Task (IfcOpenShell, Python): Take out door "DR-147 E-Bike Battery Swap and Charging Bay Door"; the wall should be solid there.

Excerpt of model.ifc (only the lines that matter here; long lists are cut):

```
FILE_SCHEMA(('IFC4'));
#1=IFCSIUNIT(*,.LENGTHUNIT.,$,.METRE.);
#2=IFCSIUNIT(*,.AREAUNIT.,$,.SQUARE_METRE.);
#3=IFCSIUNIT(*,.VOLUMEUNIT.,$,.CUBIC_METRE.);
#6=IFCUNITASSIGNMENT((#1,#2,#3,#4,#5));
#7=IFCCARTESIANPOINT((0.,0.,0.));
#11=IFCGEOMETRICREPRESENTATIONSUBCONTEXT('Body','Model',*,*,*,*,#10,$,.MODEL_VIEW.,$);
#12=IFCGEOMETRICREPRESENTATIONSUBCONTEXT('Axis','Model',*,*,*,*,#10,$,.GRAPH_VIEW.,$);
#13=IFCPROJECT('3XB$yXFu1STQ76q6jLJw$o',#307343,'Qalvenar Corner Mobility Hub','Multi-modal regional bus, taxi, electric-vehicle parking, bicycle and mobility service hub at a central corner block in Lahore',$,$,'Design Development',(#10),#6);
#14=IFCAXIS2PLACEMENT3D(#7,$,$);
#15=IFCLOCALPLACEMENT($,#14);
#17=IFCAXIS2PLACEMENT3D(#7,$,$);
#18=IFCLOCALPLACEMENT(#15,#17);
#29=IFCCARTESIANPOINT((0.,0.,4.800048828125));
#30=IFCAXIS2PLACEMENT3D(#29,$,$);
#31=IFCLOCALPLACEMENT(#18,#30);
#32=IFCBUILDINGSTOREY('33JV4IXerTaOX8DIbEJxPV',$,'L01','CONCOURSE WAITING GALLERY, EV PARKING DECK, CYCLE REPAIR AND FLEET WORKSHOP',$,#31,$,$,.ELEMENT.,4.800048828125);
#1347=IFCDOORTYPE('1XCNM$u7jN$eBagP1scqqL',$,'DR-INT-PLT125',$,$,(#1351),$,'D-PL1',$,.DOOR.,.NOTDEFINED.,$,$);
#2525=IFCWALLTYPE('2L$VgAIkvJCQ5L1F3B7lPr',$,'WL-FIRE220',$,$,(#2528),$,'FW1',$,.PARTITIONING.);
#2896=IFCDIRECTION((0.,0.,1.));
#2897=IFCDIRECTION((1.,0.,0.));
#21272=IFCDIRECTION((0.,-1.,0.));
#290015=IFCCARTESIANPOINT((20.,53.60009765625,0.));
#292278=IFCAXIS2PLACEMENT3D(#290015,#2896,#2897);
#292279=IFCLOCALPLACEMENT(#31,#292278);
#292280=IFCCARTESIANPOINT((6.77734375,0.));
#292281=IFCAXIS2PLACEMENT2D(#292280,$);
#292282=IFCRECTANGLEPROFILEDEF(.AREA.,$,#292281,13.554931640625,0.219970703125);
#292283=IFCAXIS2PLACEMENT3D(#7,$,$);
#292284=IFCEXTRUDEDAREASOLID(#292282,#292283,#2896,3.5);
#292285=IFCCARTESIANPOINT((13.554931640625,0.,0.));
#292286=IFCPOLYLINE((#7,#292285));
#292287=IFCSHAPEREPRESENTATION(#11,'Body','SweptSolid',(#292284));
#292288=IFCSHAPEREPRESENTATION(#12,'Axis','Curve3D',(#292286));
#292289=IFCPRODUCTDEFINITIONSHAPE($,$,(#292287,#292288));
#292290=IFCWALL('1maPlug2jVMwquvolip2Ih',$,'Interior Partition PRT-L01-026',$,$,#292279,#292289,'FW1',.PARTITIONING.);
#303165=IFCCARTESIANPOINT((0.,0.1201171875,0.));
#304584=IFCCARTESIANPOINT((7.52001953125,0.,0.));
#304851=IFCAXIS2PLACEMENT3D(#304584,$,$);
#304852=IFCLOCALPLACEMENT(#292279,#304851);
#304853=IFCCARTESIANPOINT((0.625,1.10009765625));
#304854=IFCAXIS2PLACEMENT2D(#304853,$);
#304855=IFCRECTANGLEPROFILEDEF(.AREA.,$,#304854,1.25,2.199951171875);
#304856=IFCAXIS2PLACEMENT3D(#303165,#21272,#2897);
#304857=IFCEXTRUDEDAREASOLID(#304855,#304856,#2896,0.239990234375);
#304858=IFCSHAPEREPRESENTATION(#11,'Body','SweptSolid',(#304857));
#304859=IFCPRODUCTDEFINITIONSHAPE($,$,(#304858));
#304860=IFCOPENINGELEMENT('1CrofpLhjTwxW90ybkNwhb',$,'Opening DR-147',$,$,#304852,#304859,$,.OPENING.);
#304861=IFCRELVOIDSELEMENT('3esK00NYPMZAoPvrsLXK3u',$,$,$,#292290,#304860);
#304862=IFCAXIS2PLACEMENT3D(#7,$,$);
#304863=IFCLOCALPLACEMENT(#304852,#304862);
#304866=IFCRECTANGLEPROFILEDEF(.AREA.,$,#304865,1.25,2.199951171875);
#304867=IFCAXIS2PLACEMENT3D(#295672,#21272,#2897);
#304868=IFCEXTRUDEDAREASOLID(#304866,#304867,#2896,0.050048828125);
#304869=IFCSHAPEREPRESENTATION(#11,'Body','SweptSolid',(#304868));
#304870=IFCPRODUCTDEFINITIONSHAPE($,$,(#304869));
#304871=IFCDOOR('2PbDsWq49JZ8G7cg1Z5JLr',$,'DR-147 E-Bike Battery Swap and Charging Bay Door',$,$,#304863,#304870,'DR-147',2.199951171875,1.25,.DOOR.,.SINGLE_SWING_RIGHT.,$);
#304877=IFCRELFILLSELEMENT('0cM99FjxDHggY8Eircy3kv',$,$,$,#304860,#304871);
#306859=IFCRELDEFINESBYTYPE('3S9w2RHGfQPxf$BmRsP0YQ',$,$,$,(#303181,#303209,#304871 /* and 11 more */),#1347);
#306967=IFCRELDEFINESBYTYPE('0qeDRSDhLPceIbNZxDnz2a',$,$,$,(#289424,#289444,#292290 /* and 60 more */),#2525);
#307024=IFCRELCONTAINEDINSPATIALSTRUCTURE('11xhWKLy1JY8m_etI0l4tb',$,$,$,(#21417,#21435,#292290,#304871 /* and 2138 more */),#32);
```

```python
import ifcopenshell
import ifcopenshell.api.feature
import ifcopenshell.api.root
import ifcopenshell.geom
import ifcopenshell.util.shape

model = ifcopenshell.open("model.ifc")
settings = ifcopenshell.geom.settings()


def volume(element):
    """Net volume in cubic metres, openings subtracted."""
    shape = ifcopenshell.geom.create_shape(settings, element)
    return ifcopenshell.util.shape.get_volume(shape.geometry)


door = model.by_guid("2PbDsWq49JZ8G7cg1Z5JLr")
opening = door.FillsVoids[0].RelatingOpeningElement
wall = opening.VoidsElements[0].RelatingBuildingElement
before = volume(wall)

ifcopenshell.api.root.remove_product(model, product=door)
ifcopenshell.api.feature.remove_feature(model, feature=opening)

after = volume(wall)

print(f"wall volume {before:.3f} -> {after:.3f} m3")

model.write("model_v2.ifc")
```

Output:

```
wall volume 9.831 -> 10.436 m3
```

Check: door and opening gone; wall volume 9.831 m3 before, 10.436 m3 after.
